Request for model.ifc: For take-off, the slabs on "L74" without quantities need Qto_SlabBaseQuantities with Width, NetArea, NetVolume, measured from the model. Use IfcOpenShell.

First a look at what the model holds.

```python
import ifcopenshell
import ifcopenshell.util.element
import ifcopenshell.util.unit

model = ifcopenshell.open("model.ifc")
print(model.schema)
for unit_type in ("LENGTHUNIT", "AREAUNIT", "VOLUMEUNIT"):
    print(unit_type, ifcopenshell.util.unit.calculate_unit_scale(model, unit_type))
storey = next(s for s in model.by_type("IfcBuildingStorey") if s.Name == "L74")
slabs = [e for e in ifcopenshell.util.element.get_decomposition(storey) if e.is_a("IfcSlab")]
for e in sorted(slabs, key=lambda e: e.id()):
    print(e.id(), e.is_a(), e.Name, list(ifcopenshell.util.element.get_psets(e, qtos_only=True)), sep=" | ")
```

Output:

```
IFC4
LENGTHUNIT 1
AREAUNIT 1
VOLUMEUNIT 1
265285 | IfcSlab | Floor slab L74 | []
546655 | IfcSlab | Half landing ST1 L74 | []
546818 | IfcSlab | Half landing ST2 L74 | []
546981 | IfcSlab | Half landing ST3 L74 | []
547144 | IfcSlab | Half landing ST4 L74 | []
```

```python
import ifcopenshell
import ifcopenshell.api.pset
import ifcopenshell.geom
import ifcopenshell.util.element
import ifcopenshell.util.shape
import ifcopenshell.util.unit

model = ifcopenshell.open("model.ifc")
unit_scale = ifcopenshell.util.unit.calculate_unit_scale(model)
area_scale = ifcopenshell.util.unit.calculate_unit_scale(model, "AREAUNIT")
volume_scale = ifcopenshell.util.unit.calculate_unit_scale(model, "VOLUMEUNIT")
settings = ifcopenshell.geom.settings()

storey = next(s for s in model.by_type("IfcBuildingStorey") if s.Name == "L74")
slabs = [e for e in ifcopenshell.util.element.get_decomposition(storey) if e.is_a("IfcSlab")]

for e in sorted(slabs, key=lambda e: e.id()):
    if ifcopenshell.util.element.get_psets(e, qtos_only=True, should_inherit=False):
        continue
    # Geometry comes back in metres, in the element's own axes.
    shape = ifcopenshell.geom.create_shape(settings, e)
    values = {
        "Width": ifcopenshell.util.shape.get_z(shape.geometry) / unit_scale,
        "NetArea": ifcopenshell.util.shape.get_footprint_area(shape.geometry) / area_scale,
        "NetVolume": ifcopenshell.util.shape.get_volume(shape.geometry) / volume_scale,
    }
    qto = ifcopenshell.api.pset.add_qto(model, product=e, name="Qto_SlabBaseQuantities")
    ifcopenshell.api.pset.edit_qto(model, qto=qto, properties=values)
    print(e.id(), {k: round(v, 3) for k, v in values.items()})

model.write("model_updated.ifc")
```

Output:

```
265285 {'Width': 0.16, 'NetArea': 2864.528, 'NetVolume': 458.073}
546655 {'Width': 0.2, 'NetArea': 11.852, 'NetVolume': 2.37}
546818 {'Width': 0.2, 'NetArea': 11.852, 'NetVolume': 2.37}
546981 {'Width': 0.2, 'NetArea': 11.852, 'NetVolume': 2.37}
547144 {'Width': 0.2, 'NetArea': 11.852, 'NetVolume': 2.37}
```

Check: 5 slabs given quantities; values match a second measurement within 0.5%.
